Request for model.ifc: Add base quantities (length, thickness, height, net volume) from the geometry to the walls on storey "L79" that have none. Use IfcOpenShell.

First a look at what the model holds.

```python
import ifcopenshell
import ifcopenshell.util.element
import ifcopenshell.util.unit

model = ifcopenshell.open("model.ifc")
print(model.schema)
for unit_type in ("LENGTHUNIT", "AREAUNIT", "VOLUMEUNIT"):
    print(unit_type, ifcopenshell.util.unit.calculate_unit_scale(model, unit_type))
storey = next(s for s in model.by_type("IfcBuildingStorey") if s.Name == "L79")
walls = [e for e in ifcopenshell.util.element.get_decomposition(storey) if e.is_a("IfcWall")]
for e in sorted(walls, key=lambda e: e.id()):
    print(e.id(), e.is_a(), e.Name, list(ifcopenshell.util.element.get_psets(e, qtos_only=True)), sep=" | ")
```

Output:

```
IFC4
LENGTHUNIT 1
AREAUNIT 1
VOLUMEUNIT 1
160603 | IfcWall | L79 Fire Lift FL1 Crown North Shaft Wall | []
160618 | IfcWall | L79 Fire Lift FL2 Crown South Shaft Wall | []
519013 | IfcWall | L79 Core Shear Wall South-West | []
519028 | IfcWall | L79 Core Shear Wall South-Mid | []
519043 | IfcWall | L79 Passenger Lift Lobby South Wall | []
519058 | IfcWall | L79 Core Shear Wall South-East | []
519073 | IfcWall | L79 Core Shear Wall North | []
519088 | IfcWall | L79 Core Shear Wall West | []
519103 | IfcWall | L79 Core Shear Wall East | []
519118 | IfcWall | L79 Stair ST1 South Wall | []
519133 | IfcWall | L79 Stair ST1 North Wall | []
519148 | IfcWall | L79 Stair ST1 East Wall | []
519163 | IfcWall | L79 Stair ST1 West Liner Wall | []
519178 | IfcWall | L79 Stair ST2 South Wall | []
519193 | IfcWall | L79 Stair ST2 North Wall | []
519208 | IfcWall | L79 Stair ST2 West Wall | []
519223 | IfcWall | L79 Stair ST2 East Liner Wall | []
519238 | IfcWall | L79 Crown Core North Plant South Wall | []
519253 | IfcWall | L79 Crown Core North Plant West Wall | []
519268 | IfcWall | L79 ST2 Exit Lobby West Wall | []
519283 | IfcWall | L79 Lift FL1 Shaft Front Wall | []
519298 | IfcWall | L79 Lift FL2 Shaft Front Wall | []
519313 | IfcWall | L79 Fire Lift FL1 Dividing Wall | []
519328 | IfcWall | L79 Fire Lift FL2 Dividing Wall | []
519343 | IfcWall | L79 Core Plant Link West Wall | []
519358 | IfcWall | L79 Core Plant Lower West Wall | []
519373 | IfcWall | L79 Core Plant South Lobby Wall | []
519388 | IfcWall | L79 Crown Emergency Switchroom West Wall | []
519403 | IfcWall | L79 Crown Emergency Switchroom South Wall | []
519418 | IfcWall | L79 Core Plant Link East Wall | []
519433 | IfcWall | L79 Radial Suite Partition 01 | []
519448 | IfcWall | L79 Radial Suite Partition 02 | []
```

```python
import ifcopenshell
import ifcopenshell.api.pset
import ifcopenshell.geom
import ifcopenshell.util.element
import ifcopenshell.util.shape
import ifcopenshell.util.unit

model = ifcopenshell.open("model.ifc")
unit_scale = ifcopenshell.util.unit.calculate_unit_scale(model)
volume_scale = ifcopenshell.util.unit.calculate_unit_scale(model, "VOLUMEUNIT")
settings = ifcopenshell.geom.settings()

storey = next(s for s in model.by_type("IfcBuildingStorey") if s.Name == "L79")
walls = [e for e in ifcopenshell.util.element.get_decomposition(storey) if e.is_a("IfcWall")]

for e in sorted(walls, key=lambda e: e.id()):
    if ifcopenshell.util.element.get_psets(e, qtos_only=True, should_inherit=False):
        continue
    # Geometry comes back in metres, in the element's own axes.
    shape = ifcopenshell.geom.create_shape(settings, e)
    values = {
        "Length": ifcopenshell.util.shape.get_x(shape.geometry) / unit_scale,
        "Width": ifcopenshell.util.shape.get_y(shape.geometry) / unit_scale,
        "Height": ifcopenshell.util.shape.get_z(shape.geometry) / unit_scale,
        "NetVolume": ifcopenshell.util.shape.get_volume(shape.geometry) / volume_scale,
    }
    qto = ifcopenshell.api.pset.add_qto(model, product=e, name="Qto_WallBaseQuantities")
    ifcopenshell.api.pset.edit_qto(model, qto=qto, properties=values)
    print(e.id(), {k: round(v, 3) for k, v in values.items()})

model.write("model_updated.ifc")
```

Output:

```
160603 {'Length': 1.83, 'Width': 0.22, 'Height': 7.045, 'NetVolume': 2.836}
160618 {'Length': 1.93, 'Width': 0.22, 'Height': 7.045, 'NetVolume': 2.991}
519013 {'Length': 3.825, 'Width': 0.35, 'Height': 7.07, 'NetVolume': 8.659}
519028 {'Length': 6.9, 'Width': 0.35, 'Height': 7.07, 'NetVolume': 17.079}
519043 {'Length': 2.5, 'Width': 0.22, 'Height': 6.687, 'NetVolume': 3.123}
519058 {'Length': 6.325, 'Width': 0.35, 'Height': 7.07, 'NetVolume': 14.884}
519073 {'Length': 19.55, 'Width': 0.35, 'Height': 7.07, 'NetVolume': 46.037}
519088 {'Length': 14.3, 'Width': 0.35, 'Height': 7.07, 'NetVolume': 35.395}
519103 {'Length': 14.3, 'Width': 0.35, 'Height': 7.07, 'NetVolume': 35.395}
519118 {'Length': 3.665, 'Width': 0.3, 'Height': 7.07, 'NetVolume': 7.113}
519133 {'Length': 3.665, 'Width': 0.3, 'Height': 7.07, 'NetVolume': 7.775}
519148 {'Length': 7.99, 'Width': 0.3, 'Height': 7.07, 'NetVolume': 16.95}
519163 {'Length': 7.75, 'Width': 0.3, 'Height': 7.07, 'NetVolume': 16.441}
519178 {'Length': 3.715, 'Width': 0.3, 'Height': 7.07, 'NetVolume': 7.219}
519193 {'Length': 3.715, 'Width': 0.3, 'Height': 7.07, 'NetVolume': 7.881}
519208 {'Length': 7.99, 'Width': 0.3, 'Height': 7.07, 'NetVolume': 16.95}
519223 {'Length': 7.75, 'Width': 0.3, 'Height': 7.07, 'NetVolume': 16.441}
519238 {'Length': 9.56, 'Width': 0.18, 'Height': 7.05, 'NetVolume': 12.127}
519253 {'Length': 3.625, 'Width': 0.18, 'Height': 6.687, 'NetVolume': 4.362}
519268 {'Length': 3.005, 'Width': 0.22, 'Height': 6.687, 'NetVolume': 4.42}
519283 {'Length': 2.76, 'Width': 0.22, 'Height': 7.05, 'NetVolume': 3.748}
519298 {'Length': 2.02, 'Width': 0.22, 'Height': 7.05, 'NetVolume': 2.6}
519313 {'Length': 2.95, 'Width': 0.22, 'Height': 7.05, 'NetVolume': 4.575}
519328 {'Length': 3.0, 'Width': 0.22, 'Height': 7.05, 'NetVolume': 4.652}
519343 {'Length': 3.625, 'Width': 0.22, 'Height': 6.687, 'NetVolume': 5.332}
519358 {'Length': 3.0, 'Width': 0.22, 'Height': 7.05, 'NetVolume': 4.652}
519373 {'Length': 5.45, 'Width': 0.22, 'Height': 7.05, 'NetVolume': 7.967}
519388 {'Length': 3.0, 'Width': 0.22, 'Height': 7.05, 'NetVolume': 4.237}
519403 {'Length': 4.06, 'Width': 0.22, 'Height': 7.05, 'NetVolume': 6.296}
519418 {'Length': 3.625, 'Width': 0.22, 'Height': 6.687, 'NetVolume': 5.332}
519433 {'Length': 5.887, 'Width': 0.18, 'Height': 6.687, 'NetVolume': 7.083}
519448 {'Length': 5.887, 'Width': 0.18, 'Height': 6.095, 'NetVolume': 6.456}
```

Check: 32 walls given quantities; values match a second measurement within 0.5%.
